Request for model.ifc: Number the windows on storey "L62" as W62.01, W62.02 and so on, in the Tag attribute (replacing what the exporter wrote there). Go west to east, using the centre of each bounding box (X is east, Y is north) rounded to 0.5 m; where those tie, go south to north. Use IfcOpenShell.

First a look at what the model holds.

```python
import ifcopenshell
import ifcopenshell.util.element
import ifcopenshell.util.placement

model = ifcopenshell.open("model.ifc")
print(model.schema)
storey = next(s for s in model.by_type("IfcBuildingStorey") if s.Name == "L62")
windows = [e for e in ifcopenshell.util.element.get_decomposition(storey) if e.is_a("IfcWindow")]
for e in sorted(windows, key=lambda e: e.id()):
    origin = ifcopenshell.util.placement.get_local_placement(e.ObjectPlacement)[:3, 3]
    print(e.id(), e.Tag, e.Name, origin.round(2) + 0.0, sep=" | ")
```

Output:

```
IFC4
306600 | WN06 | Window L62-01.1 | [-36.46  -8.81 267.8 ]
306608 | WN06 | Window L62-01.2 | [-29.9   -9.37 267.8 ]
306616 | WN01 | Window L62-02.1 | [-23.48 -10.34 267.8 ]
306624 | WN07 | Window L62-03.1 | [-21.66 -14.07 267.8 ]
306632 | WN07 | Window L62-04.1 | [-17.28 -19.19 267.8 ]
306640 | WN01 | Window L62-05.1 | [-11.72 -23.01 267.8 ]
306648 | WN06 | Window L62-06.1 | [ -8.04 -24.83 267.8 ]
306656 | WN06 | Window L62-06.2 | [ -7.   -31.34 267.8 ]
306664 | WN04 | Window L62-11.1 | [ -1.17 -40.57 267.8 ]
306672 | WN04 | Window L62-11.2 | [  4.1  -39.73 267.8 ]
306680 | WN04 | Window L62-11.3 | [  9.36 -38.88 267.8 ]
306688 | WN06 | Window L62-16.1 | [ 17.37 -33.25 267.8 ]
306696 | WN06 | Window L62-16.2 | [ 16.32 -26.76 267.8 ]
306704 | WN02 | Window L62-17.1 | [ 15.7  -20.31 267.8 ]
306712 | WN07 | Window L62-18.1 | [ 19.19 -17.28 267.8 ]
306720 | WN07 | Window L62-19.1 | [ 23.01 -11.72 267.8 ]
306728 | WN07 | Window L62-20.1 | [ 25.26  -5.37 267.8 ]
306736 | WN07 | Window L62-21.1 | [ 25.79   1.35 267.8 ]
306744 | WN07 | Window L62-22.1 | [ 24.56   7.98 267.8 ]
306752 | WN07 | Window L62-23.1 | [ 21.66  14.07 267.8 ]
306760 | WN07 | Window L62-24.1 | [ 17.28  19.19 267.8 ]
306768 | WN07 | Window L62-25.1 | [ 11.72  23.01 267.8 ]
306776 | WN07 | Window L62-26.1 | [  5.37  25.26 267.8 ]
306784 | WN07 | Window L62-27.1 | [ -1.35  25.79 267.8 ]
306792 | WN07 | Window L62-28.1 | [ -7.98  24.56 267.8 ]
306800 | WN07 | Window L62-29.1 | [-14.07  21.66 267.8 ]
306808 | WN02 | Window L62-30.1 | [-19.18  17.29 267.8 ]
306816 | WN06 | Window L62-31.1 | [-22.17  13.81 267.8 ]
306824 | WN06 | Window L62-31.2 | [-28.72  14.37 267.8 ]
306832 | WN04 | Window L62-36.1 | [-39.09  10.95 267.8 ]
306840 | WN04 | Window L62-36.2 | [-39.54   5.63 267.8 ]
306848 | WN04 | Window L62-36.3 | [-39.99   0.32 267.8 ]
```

```python
import ifcopenshell
import ifcopenshell.geom
import ifcopenshell.util.element
import ifcopenshell.util.shape

model = ifcopenshell.open("model.ifc")
settings = ifcopenshell.geom.settings()
settings.set("use-world-coords", True)


def centre(element):
    shape = ifcopenshell.geom.create_shape(settings, element)
    return ifcopenshell.util.shape.get_bbox_centroid(shape.geometry)


storey = next(s for s in model.by_type("IfcBuildingStorey") if s.Name == "L62")
windows = [e for e in ifcopenshell.util.element.get_decomposition(storey) if e.is_a("IfcWindow")]

# Insertion points can sit at a corner or the storey origin, so sort by the geometry (in metres).
centres = {e: centre(e) for e in windows}
windows.sort(key=lambda e: (round(centres[e][0] / 0.5), centres[e][1]))

for i, e in enumerate(windows, start=1):
    number = f"W62.{i:02d}"
    e.Tag = number
    print(e.id(), number)

model.write("model-out.ifc")
```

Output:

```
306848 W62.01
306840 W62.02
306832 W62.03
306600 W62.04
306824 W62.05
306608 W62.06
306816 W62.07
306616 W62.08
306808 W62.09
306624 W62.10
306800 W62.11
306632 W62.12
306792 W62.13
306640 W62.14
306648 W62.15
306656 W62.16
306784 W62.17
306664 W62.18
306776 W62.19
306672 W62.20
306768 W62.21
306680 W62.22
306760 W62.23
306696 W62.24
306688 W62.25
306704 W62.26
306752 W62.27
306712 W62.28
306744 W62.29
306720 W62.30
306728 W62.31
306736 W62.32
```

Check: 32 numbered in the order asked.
